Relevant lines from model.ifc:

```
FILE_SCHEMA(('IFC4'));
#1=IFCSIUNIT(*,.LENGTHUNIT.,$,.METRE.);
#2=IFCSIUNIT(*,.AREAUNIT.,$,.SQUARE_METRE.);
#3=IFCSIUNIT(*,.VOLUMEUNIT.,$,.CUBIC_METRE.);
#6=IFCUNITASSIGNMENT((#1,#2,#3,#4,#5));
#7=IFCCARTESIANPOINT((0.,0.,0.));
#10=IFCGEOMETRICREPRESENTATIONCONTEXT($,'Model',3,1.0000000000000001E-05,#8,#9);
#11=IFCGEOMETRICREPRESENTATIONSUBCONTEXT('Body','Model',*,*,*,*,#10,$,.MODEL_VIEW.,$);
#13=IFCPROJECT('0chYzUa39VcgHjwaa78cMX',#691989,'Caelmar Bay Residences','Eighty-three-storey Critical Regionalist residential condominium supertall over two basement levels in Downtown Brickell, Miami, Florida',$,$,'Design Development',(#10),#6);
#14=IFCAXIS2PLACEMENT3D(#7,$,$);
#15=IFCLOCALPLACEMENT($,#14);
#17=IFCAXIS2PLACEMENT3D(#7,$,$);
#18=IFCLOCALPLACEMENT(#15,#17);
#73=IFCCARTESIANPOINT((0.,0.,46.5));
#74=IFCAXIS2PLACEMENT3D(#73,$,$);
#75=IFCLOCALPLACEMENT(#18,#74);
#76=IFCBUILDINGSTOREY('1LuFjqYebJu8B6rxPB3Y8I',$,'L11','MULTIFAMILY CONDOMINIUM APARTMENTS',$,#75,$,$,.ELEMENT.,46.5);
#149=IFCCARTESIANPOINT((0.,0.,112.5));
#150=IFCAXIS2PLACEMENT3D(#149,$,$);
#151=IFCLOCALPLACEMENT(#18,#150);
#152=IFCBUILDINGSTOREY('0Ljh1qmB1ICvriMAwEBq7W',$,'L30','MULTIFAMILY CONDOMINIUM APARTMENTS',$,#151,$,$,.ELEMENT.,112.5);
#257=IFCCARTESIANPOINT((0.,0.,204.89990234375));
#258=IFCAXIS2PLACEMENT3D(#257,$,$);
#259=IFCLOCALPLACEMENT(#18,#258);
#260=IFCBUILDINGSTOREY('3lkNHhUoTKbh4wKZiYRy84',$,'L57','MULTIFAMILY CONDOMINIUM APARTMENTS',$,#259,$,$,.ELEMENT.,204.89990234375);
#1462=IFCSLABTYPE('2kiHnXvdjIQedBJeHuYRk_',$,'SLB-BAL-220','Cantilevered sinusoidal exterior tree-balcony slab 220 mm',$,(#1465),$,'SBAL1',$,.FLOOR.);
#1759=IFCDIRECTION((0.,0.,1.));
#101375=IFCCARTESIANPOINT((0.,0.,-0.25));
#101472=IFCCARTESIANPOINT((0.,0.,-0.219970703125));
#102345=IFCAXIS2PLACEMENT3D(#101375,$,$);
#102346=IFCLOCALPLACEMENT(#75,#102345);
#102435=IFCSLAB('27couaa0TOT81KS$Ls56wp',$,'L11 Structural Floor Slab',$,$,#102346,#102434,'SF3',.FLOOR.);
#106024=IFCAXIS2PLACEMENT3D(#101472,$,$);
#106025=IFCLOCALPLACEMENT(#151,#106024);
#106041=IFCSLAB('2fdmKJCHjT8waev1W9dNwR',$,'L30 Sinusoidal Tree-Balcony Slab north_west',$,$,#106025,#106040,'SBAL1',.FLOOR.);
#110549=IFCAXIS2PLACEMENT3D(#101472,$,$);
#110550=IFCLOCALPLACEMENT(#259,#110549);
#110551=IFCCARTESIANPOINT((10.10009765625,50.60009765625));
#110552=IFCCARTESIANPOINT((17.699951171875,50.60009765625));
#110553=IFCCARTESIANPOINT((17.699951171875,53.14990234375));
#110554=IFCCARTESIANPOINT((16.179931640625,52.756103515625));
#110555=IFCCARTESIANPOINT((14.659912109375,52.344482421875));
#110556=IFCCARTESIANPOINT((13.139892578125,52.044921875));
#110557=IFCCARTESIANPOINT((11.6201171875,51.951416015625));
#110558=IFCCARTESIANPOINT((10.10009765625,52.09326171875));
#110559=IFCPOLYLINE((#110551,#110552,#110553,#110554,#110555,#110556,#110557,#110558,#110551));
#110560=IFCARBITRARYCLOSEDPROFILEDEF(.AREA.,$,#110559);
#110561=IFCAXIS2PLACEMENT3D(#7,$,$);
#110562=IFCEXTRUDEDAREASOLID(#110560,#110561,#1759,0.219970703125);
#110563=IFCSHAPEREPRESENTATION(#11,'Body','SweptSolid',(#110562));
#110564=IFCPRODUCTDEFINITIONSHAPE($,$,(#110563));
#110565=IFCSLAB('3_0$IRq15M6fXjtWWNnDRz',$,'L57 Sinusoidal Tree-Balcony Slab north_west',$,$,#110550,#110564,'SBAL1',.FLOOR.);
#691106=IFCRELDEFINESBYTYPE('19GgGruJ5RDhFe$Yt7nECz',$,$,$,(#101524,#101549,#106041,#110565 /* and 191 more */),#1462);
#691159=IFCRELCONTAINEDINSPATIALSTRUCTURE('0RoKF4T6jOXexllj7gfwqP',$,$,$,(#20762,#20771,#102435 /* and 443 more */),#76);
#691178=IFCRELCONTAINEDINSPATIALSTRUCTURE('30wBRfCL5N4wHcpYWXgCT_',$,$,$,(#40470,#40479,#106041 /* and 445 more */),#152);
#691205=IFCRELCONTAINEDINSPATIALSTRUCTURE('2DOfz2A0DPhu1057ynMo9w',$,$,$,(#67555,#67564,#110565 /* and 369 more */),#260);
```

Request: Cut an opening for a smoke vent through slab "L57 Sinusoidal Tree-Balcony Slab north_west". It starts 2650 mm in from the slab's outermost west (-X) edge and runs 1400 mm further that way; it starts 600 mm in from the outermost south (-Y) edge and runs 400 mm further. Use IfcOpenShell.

```python
import numpy as np
import ifcopenshell
import ifcopenshell.api.feature
import ifcopenshell.api.geometry
import ifcopenshell.api.root
import ifcopenshell.geom
import ifcopenshell.util.placement
import ifcopenshell.util.representation
import ifcopenshell.util.shape
import ifcopenshell.util.unit

model = ifcopenshell.open("model.ifc")
unit_scale = ifcopenshell.util.unit.calculate_unit_scale(model)
settings = ifcopenshell.geom.settings()


def volume(element):
    """Net volume in cubic metres, openings subtracted."""
    shape = ifcopenshell.geom.create_shape(settings, element)
    return ifcopenshell.util.shape.get_volume(shape.geometry)


slab = model.by_guid("3_0$IRq15M6fXjtWWNnDRz")
before = volume(slab)

# Extent in the slab's own axes, in metres. The edges named are its -X and -Y sides.
slab_shape = ifcopenshell.geom.create_shape(settings, slab)
vertices = ifcopenshell.util.shape.get_vertices(slab_shape.geometry)
x_min, y_min, bottom = vertices.min(axis=0)
top = vertices[:, 2].max()

opening = ifcopenshell.api.root.create_entity(model, ifc_class="IfcOpeningElement", name="Smoke vent opening", predefined_type="OPENING")
context = ifcopenshell.util.representation.get_context(model, "Model", "Body", "MODEL_VIEW")
width, depth = 1.4, 0.4
outline = [(0.0, 0.0), (width, 0.0), (width, depth), (0.0, depth), (0.0, 0.0)]
# Overshoot both faces by 50 mm so the cut is clean.
shape = ifcopenshell.api.geometry.add_slab_representation(
    model, context=context, depth=top - bottom + 0.1, polyline=outline
)
ifcopenshell.api.geometry.assign_representation(model, product=opening, representation=shape)

matrix = ifcopenshell.util.placement.get_local_placement(slab.ObjectPlacement)
matrix[:, 3] = matrix @ np.append(np.array([x_min + 2.65, y_min + 0.6, bottom - 0.05]) / unit_scale, 1.0)
ifcopenshell.api.geometry.edit_object_placement(model, product=opening, matrix=matrix, is_si=False)
ifcopenshell.api.feature.add_feature(model, feature=opening, element=slab)

after = volume(slab)

print(f"slab volume {before:.3f} -> {after:.3f} m3")

model.write("model_edited.ifc")
```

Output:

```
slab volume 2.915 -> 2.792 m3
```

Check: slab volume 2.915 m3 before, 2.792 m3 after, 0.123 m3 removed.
